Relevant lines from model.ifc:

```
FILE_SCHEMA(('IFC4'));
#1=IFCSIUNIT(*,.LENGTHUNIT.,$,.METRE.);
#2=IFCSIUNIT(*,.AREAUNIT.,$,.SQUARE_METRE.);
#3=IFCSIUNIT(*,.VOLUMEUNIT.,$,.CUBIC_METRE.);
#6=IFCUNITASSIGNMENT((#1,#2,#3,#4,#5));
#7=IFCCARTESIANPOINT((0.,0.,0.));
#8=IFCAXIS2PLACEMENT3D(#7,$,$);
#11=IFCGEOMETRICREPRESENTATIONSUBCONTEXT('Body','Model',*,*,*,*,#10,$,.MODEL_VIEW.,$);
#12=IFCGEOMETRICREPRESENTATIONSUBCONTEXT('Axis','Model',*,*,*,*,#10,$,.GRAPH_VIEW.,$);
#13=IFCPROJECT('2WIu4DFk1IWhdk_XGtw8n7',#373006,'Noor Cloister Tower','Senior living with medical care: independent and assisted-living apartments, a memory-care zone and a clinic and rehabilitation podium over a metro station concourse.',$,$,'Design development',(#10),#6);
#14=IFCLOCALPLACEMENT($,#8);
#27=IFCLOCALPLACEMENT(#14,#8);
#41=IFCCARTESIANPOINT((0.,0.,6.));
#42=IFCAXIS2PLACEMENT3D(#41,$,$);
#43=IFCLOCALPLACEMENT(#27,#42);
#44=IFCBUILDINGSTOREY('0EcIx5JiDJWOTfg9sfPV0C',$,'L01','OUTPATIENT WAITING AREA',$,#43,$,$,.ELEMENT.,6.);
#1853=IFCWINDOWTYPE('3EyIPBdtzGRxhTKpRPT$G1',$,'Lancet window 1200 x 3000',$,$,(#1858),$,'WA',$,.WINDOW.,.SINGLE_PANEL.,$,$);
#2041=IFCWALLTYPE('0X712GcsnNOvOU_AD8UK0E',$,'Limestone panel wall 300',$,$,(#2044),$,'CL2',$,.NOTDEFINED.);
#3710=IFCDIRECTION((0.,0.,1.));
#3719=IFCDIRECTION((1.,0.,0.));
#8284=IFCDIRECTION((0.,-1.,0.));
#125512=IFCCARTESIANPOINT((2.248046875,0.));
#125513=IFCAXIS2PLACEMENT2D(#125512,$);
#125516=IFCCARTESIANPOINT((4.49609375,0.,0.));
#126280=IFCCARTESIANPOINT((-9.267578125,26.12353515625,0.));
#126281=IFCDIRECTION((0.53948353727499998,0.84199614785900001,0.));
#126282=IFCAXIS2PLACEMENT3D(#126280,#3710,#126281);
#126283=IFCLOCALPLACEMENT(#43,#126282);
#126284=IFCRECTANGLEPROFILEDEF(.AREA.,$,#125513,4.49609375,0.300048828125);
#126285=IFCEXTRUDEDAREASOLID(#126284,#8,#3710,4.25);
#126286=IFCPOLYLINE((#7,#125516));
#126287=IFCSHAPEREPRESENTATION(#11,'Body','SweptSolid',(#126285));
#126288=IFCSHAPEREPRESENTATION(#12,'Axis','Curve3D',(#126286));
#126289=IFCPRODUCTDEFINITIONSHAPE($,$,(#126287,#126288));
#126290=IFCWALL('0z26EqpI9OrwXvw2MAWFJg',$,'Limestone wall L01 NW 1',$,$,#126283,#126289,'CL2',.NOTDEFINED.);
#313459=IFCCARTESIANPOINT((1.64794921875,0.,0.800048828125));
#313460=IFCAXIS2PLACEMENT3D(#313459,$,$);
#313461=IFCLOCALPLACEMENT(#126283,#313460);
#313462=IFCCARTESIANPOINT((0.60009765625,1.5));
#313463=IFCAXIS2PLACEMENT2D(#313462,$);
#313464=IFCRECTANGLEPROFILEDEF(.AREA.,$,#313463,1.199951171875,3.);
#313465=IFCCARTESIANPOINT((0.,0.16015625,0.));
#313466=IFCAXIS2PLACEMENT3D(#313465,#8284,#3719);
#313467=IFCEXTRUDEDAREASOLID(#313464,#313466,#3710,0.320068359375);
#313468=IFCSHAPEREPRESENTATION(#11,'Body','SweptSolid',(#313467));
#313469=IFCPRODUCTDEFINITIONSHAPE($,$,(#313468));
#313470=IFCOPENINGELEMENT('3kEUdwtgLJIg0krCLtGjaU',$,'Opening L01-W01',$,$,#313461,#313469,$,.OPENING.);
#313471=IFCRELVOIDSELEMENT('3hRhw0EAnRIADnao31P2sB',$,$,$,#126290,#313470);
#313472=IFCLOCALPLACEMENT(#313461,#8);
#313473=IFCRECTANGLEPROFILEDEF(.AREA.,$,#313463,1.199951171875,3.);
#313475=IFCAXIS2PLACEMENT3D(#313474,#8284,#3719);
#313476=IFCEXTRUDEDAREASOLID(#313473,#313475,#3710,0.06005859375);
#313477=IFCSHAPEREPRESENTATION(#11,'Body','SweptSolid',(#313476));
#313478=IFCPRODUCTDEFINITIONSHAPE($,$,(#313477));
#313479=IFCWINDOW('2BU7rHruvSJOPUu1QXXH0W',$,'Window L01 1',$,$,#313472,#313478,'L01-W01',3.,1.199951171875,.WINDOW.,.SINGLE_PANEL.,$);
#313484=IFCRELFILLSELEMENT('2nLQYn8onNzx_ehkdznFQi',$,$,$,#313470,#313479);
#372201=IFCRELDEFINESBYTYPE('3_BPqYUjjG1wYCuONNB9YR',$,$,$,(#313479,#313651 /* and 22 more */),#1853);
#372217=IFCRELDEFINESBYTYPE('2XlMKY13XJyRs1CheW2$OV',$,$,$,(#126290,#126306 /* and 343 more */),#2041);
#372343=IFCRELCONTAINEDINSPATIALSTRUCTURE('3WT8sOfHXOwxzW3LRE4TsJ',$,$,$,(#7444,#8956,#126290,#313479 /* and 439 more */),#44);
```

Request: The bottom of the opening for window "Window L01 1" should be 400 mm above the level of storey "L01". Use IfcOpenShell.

```python
import numpy as np
import ifcopenshell
import ifcopenshell.api.geometry
import ifcopenshell.geom
import ifcopenshell.util.element
import ifcopenshell.util.placement
import ifcopenshell.util.shape
import ifcopenshell.util.unit

model = ifcopenshell.open("model.ifc")
unit_scale = ifcopenshell.util.unit.calculate_unit_scale(model)

window = model.by_guid("2BU7rHruvSJOPUu1QXXH0W")
opening = window.FillsVoids[0].RelatingOpeningElement
storey = ifcopenshell.util.element.get_container(window, ifc_class="IfcBuildingStorey")
level = ifcopenshell.util.placement.get_local_placement(storey.ObjectPlacement)[2, 3]

# The opening's origin need not be at the sill, so measure its lowest point.
shape = ifcopenshell.geom.create_shape(ifcopenshell.geom.settings(), opening)
bottom = ifcopenshell.util.shape.get_shape_bottom_elevation(shape, shape.geometry) / unit_scale
dz = level + 0.4 - bottom

shift = np.array([0.0, 0.0, dz])
# The window is placed relative to its opening, so it follows when the opening moves.
matrix = ifcopenshell.util.placement.get_local_placement(opening.ObjectPlacement)
matrix[:3, 3] += shift
ifcopenshell.api.geometry.edit_object_placement(
    model, product=opening, matrix=matrix, is_si=False, should_transform_children=True
)

print(f"moved by {dz * unit_scale:+.3f} m")

model.write("model_v2.ifc")
```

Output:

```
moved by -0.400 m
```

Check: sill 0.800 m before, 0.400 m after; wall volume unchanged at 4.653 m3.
